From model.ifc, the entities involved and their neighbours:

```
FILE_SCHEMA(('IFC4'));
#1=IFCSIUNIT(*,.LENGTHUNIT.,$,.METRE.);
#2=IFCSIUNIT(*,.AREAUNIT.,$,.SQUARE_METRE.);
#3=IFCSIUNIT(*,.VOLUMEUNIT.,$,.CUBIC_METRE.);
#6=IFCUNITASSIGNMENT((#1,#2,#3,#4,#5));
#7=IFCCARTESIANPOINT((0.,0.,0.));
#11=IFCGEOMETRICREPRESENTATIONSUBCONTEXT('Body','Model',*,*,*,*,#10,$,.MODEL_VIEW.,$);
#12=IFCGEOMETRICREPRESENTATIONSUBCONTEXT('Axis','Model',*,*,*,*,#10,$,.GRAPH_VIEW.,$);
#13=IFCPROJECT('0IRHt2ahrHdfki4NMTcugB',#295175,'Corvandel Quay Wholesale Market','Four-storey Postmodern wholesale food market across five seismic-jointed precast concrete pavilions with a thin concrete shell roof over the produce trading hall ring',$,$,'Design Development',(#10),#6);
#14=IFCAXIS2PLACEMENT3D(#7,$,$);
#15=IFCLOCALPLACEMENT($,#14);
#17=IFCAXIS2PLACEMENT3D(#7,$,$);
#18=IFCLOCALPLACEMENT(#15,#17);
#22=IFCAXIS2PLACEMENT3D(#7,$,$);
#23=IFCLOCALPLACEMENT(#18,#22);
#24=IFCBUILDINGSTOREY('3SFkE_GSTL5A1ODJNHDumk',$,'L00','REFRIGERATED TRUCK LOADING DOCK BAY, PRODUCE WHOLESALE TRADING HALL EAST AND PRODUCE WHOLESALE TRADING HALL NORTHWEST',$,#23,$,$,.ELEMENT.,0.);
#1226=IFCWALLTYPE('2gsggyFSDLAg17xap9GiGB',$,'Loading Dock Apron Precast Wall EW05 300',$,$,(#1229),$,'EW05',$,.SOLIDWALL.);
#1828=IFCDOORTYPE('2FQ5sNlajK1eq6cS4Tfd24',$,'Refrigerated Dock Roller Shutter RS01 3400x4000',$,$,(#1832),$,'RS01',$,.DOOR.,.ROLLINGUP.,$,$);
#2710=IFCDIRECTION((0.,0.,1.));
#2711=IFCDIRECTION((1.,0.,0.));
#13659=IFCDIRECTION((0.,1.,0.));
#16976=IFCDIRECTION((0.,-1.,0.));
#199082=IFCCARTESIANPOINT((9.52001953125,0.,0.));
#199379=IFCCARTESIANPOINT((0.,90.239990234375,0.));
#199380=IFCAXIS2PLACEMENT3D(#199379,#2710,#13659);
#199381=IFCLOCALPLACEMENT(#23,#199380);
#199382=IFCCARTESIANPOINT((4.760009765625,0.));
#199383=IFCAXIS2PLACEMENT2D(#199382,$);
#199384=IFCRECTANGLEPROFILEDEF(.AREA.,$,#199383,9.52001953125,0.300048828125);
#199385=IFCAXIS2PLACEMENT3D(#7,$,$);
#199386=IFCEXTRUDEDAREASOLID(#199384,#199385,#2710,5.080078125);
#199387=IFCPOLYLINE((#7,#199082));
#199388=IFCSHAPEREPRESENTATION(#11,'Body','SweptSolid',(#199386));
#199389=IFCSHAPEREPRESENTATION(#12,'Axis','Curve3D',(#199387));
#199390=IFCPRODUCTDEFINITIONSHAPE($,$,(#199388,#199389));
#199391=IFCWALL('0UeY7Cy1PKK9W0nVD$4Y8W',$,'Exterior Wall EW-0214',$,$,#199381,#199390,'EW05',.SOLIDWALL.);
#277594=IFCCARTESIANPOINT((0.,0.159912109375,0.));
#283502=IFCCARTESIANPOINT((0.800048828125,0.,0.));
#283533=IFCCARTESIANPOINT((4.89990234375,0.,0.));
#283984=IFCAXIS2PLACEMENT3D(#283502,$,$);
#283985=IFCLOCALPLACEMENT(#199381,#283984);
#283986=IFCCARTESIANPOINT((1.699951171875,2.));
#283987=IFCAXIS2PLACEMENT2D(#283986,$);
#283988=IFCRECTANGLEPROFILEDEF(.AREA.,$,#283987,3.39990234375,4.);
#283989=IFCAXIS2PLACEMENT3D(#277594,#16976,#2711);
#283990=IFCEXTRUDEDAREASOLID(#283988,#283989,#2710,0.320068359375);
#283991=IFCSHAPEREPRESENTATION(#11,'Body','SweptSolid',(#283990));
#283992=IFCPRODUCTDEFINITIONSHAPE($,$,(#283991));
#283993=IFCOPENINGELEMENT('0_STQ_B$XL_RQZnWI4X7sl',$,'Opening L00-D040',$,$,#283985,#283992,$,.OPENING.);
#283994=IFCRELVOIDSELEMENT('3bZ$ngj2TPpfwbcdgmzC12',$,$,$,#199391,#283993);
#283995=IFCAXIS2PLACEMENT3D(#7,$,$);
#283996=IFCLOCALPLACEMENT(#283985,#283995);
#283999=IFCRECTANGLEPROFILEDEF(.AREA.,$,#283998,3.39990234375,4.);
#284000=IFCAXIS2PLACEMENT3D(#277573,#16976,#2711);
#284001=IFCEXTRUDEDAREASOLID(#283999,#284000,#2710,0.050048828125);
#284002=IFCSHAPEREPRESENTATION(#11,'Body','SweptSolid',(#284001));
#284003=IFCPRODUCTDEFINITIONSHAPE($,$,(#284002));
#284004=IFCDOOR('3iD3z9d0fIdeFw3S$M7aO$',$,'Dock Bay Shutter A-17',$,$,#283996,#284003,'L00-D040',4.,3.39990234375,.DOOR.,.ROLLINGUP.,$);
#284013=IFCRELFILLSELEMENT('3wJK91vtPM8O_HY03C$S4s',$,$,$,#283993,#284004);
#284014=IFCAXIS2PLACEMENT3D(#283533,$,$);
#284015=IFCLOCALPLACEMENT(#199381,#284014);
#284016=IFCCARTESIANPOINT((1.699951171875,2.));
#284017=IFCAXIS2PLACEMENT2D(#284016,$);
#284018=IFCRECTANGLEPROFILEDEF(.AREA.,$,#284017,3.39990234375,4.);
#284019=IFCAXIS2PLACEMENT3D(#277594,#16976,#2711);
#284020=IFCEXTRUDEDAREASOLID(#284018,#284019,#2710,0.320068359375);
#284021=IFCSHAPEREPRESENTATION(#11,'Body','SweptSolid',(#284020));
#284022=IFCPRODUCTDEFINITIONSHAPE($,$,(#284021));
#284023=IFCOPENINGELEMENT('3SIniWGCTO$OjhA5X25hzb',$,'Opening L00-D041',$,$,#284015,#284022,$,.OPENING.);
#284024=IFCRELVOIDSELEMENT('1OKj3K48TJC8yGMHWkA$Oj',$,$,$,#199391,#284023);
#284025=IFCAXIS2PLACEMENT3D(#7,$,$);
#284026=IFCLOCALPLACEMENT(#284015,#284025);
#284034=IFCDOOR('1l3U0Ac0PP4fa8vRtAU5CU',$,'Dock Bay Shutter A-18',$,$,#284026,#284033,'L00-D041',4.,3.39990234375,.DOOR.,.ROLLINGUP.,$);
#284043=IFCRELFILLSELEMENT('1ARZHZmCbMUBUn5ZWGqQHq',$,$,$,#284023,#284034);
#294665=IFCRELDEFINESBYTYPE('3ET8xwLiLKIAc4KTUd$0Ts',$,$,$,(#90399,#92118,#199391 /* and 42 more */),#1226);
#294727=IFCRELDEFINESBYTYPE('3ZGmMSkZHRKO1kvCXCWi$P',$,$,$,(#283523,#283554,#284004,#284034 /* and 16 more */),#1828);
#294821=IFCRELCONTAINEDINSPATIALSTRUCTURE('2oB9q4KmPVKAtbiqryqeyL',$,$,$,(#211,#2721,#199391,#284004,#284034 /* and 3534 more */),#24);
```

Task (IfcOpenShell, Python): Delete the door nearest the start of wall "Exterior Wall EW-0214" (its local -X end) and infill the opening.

```python
import ifcopenshell
import ifcopenshell.api.feature
import ifcopenshell.api.root
import ifcopenshell.geom
import ifcopenshell.util.shape

model = ifcopenshell.open("model.ifc")
settings = ifcopenshell.geom.settings()


def volume(element):
    """Net volume in cubic metres, openings subtracted."""
    shape = ifcopenshell.geom.create_shape(settings, element)
    return ifcopenshell.util.shape.get_volume(shape.geometry)


door = model.by_guid("3iD3z9d0fIdeFw3S$M7aO$")
opening = door.FillsVoids[0].RelatingOpeningElement
wall = opening.VoidsElements[0].RelatingBuildingElement
before = volume(wall)

ifcopenshell.api.root.remove_product(model, product=door)
ifcopenshell.api.feature.remove_feature(model, feature=opening)

after = volume(wall)

print(f"wall volume {before:.3f} -> {after:.3f} m3")

model.write("model_updated.ifc")
```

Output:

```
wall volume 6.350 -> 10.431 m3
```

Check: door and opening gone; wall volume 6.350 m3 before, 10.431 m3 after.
